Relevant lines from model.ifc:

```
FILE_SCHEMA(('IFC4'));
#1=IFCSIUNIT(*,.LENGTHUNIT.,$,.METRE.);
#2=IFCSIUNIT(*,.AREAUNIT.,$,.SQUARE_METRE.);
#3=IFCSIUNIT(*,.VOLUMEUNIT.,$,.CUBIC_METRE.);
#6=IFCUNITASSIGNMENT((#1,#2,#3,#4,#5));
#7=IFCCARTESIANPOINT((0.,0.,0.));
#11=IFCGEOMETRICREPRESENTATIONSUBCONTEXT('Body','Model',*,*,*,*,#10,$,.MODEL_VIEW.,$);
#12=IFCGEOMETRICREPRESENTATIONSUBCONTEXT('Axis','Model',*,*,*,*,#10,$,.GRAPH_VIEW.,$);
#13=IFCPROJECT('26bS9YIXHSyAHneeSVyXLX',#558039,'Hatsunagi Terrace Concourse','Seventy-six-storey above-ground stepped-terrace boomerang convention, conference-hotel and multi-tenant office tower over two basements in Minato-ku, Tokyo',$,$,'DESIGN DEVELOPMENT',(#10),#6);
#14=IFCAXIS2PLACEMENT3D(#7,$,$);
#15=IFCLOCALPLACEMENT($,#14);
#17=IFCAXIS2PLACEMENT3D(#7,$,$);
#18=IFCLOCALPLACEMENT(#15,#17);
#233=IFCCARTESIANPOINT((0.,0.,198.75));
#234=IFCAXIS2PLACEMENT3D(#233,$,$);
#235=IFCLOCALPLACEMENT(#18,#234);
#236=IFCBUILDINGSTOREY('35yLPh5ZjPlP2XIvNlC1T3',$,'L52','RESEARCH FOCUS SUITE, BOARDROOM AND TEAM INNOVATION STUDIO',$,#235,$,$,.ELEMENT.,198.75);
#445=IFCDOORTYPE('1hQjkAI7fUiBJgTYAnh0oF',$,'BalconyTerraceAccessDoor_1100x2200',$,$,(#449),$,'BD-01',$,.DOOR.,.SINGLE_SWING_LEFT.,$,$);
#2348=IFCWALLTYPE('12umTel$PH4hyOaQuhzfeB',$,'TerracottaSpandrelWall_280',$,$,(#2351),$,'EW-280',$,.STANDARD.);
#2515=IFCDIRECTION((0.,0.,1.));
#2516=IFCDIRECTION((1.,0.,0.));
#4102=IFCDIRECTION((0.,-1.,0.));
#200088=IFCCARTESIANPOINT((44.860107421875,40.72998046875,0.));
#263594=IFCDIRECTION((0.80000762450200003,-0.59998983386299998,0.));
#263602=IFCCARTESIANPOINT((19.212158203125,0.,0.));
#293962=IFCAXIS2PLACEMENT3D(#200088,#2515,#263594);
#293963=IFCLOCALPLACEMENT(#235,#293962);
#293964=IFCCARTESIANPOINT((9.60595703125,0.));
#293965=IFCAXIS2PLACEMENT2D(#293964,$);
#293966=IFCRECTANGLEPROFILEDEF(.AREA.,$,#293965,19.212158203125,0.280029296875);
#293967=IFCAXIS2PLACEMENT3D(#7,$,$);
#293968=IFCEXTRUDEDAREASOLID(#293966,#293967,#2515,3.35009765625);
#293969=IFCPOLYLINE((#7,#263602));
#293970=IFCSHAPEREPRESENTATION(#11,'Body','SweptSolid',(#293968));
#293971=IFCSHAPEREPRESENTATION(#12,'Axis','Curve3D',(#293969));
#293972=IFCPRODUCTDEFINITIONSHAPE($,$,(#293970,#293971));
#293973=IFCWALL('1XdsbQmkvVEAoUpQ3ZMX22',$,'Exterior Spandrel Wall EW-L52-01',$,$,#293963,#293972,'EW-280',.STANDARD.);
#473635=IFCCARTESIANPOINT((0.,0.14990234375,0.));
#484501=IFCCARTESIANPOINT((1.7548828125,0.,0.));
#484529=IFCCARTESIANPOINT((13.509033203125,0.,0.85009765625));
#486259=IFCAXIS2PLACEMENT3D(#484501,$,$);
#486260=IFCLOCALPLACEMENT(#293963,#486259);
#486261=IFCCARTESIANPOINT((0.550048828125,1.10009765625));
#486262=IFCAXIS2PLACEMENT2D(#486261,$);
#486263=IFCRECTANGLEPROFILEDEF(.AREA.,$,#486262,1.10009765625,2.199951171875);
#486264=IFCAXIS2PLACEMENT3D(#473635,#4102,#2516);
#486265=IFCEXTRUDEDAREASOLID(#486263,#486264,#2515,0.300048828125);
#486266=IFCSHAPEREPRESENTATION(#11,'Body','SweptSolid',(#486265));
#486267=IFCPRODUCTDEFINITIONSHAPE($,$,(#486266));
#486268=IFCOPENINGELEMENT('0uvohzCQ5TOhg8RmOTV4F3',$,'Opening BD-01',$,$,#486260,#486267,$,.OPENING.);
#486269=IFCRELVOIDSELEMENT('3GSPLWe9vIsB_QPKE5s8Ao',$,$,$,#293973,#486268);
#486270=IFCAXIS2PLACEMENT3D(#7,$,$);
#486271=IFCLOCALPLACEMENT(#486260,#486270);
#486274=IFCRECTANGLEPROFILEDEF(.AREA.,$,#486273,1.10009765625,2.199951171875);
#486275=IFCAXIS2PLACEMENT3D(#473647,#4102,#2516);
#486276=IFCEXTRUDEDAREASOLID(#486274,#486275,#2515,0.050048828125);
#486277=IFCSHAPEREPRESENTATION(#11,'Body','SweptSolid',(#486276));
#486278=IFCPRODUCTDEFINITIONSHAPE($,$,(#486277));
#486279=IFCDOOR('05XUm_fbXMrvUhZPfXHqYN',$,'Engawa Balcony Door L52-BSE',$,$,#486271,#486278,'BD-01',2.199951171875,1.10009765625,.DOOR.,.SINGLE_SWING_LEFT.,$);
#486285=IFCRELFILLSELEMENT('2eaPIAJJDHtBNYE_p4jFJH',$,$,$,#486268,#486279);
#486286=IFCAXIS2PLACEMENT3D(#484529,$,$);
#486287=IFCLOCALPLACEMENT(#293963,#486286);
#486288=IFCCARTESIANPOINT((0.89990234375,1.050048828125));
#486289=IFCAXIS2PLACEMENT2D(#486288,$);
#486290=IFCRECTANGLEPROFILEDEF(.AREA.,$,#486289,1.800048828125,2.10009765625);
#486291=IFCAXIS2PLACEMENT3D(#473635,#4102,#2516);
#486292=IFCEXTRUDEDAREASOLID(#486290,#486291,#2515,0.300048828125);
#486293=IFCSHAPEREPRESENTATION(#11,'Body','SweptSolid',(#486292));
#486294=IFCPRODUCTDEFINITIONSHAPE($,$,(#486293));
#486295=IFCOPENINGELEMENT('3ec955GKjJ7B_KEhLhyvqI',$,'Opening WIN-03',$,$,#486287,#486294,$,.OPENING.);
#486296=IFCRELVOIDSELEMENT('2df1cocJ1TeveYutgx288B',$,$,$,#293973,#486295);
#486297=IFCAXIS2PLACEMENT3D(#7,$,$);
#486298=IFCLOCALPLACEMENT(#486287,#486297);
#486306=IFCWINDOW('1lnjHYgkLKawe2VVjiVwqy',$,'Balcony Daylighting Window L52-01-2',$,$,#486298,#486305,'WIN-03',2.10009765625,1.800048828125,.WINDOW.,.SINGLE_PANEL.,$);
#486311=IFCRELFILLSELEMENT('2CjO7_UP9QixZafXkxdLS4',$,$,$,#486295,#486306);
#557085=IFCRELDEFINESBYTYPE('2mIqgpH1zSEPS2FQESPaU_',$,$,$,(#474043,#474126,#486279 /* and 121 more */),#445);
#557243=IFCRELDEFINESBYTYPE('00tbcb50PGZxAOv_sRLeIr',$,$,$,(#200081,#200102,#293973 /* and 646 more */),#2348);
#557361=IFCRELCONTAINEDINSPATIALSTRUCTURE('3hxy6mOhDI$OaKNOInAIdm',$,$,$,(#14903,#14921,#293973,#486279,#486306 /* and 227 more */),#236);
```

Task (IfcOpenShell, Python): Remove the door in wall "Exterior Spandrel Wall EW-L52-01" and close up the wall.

```python
import ifcopenshell
import ifcopenshell.api.feature
import ifcopenshell.api.root
import ifcopenshell.geom
import ifcopenshell.util.shape

model = ifcopenshell.open("model.ifc")
settings = ifcopenshell.geom.settings()


def volume(element):
    """Net volume in cubic metres, openings subtracted."""
    shape = ifcopenshell.geom.create_shape(settings, element)
    return ifcopenshell.util.shape.get_volume(shape.geometry)


door = model.by_id(486279)
opening = door.FillsVoids[0].RelatingOpeningElement
wall = opening.VoidsElements[0].RelatingBuildingElement
before = volume(wall)

ifcopenshell.api.root.remove_product(model, product=door)
ifcopenshell.api.feature.remove_feature(model, feature=opening)

after = volume(wall)

print(f"wall volume {before:.3f} -> {after:.3f} m3")

model.write("model_rev.ifc")
```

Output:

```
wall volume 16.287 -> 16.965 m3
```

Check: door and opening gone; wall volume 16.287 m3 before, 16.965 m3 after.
